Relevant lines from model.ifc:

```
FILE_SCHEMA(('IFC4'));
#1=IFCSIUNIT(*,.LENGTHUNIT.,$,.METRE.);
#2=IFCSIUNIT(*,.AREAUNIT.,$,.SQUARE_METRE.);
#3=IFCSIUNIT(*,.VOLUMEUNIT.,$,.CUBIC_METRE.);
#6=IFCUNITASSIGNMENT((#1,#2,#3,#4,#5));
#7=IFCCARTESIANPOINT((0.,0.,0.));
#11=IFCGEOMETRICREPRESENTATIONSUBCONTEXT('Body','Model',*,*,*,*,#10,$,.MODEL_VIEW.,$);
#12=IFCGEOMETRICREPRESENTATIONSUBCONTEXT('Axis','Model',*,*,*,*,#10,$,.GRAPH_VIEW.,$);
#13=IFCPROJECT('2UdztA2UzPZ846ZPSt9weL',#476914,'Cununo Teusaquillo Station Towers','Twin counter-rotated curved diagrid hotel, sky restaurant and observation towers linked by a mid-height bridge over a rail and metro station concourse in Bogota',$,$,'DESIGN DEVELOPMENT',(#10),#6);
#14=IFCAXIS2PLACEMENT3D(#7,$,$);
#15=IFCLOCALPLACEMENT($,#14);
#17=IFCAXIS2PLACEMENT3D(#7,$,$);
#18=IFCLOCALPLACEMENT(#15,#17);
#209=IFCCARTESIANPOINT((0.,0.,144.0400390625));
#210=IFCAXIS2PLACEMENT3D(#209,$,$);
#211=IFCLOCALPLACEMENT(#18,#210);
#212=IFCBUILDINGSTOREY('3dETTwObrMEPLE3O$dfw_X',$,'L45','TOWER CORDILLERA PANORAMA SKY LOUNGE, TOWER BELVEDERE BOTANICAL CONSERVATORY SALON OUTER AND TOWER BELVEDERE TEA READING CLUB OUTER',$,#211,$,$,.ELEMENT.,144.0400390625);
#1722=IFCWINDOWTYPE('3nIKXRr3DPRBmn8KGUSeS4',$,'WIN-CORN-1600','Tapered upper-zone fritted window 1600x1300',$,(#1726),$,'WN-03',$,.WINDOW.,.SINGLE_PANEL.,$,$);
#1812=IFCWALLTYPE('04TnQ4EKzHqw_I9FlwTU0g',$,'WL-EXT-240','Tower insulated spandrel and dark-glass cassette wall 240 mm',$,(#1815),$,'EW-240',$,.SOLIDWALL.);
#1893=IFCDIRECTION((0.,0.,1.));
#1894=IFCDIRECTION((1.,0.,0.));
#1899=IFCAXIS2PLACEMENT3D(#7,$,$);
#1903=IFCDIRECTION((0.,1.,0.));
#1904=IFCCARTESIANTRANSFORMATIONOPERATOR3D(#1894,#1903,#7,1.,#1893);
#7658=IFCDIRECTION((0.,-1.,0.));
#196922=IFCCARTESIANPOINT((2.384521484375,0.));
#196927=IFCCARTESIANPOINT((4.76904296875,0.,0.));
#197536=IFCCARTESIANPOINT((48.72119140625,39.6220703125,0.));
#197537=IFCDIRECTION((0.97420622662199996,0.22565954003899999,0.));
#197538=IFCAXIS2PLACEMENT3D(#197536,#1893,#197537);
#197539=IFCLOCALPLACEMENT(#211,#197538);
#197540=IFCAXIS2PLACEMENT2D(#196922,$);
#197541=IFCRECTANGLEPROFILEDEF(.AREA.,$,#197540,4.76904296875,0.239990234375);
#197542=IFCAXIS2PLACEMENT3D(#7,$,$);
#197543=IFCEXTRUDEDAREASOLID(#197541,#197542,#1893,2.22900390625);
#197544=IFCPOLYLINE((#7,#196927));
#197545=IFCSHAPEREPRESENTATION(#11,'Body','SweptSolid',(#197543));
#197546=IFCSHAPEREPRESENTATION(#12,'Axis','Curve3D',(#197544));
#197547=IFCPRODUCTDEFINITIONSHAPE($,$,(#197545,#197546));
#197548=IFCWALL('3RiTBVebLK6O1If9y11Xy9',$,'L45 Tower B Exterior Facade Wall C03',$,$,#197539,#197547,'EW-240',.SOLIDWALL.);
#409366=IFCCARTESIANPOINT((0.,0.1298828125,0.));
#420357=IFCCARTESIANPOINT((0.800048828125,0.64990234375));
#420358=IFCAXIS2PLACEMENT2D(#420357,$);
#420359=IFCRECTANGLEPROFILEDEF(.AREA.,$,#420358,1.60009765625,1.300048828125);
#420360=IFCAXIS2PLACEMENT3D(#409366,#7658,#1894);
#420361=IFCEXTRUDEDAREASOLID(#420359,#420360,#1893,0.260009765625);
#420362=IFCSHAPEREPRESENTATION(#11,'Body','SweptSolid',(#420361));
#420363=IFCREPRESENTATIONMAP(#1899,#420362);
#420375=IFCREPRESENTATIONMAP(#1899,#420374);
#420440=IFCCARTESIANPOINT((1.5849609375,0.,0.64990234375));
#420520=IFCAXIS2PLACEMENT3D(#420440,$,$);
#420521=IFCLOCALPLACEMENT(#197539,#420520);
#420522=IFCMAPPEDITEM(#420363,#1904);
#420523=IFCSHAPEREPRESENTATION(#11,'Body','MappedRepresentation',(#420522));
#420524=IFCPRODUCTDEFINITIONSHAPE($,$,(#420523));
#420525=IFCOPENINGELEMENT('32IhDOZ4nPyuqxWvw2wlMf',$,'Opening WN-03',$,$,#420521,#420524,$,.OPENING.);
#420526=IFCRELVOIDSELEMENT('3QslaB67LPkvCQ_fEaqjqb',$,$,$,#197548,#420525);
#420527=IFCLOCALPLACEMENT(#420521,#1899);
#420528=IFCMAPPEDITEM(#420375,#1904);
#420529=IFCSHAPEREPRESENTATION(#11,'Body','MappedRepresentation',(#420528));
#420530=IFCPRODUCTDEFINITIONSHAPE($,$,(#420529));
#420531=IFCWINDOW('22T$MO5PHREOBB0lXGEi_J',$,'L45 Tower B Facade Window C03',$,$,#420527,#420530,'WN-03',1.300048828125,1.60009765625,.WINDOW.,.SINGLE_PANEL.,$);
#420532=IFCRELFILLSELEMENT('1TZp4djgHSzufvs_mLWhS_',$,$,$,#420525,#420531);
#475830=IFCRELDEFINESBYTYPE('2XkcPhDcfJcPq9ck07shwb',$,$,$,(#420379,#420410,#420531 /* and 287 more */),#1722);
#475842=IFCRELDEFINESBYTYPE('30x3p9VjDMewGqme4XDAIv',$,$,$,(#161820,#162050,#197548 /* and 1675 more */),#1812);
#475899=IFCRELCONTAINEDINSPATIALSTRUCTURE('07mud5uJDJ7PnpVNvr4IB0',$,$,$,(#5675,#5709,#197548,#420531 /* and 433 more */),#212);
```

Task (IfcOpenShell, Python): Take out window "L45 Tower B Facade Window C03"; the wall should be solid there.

```python
import ifcopenshell
import ifcopenshell.api.feature
import ifcopenshell.api.root
import ifcopenshell.geom
import ifcopenshell.util.shape

model = ifcopenshell.open("model.ifc")
settings = ifcopenshell.geom.settings()


def volume(element):
    """Net volume in cubic metres, openings subtracted."""
    shape = ifcopenshell.geom.create_shape(settings, element)
    return ifcopenshell.util.shape.get_volume(shape.geometry)


window = model.by_guid("22T$MO5PHREOBB0lXGEi_J")
opening = window.FillsVoids[0].RelatingOpeningElement
wall = opening.VoidsElements[0].RelatingBuildingElement
before = volume(wall)

ifcopenshell.api.root.remove_product(model, product=window)
ifcopenshell.api.feature.remove_feature(model, feature=opening)

after = volume(wall)

print(f"wall volume {before:.3f} -> {after:.3f} m3")

model.write("model_edited.ifc")
```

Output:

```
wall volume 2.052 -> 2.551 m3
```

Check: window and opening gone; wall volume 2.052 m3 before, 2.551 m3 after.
